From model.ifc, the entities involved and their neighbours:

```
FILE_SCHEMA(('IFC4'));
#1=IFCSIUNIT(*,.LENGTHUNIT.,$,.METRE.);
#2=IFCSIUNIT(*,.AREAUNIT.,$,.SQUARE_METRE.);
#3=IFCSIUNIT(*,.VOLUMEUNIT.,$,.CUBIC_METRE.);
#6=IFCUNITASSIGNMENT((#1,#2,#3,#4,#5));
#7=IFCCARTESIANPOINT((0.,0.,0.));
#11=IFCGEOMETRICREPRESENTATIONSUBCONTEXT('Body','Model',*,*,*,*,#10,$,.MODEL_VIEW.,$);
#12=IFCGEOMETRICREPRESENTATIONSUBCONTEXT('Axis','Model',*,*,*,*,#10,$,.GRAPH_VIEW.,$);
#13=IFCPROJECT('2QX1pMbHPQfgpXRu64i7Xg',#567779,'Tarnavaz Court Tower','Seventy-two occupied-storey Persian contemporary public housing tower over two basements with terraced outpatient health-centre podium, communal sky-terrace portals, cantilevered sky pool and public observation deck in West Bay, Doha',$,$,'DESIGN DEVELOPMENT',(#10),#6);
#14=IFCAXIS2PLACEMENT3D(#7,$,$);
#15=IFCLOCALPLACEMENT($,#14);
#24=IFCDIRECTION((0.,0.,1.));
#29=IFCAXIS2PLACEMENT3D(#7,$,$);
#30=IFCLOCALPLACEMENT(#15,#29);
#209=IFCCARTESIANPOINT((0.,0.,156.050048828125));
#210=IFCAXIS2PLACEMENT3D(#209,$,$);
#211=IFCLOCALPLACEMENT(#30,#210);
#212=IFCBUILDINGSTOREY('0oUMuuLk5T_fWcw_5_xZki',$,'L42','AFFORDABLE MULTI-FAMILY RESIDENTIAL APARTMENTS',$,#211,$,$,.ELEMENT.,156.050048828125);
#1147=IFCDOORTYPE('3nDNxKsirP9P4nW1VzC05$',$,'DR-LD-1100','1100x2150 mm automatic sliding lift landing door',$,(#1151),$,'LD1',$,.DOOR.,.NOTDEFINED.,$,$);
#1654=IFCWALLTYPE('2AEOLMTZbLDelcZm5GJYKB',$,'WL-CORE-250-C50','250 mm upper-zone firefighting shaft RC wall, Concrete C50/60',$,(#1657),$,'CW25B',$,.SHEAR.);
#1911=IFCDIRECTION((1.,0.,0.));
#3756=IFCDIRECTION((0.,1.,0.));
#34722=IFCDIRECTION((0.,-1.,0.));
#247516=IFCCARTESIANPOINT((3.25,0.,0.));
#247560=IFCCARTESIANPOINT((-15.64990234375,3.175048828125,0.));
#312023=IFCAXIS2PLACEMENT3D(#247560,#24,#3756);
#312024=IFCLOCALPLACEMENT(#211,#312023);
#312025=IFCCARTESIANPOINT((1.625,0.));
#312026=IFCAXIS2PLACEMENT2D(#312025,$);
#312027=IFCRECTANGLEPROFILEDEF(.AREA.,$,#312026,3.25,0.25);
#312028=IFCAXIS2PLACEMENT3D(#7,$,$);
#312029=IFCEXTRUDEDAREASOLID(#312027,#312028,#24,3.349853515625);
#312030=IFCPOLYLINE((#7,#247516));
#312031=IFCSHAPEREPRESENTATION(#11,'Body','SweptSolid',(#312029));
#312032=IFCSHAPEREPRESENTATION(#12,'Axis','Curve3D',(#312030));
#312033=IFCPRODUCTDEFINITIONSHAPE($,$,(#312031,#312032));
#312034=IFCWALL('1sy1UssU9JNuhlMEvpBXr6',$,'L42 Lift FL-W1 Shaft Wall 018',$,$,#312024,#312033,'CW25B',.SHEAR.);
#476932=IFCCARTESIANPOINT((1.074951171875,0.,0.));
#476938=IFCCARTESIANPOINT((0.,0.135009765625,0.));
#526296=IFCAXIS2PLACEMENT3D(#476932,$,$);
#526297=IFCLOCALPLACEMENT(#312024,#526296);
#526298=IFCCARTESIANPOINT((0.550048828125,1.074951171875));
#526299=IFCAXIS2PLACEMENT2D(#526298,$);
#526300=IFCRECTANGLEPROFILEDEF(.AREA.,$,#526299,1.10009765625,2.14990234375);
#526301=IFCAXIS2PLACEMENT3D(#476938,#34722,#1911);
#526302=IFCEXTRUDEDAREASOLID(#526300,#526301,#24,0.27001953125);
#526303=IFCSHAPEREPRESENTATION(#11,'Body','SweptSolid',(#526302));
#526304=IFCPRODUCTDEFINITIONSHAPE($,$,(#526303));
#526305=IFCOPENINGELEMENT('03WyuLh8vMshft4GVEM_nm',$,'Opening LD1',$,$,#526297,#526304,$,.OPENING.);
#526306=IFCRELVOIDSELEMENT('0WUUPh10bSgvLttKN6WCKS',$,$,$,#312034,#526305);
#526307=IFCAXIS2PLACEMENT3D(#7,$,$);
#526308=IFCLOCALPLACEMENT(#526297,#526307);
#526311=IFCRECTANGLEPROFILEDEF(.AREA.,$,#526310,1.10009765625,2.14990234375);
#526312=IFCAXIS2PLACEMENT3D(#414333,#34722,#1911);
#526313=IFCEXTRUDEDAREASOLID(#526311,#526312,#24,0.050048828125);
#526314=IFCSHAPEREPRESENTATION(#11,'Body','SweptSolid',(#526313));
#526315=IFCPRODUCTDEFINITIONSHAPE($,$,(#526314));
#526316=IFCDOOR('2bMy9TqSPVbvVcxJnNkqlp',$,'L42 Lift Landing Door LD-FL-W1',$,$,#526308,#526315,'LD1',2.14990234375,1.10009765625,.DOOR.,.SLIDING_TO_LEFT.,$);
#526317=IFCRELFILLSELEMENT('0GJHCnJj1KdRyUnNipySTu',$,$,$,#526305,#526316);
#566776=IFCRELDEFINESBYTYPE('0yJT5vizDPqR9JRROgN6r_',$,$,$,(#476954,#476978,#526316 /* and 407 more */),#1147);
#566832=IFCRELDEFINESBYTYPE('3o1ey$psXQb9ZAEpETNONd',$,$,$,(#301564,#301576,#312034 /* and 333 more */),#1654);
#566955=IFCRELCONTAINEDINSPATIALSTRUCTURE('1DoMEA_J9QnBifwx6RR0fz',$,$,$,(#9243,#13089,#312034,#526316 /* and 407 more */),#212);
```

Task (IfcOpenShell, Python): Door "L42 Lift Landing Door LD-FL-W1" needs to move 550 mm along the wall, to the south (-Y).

```python
import ifcopenshell
import ifcopenshell.api.geometry
import ifcopenshell.util.placement

model = ifcopenshell.open("model.ifc")

door = model.by_id(526316)
opening = door.FillsVoids[0].RelatingOpeningElement
wall = opening.VoidsElements[0].RelatingBuildingElement

wall_matrix = ifcopenshell.util.placement.get_local_placement(wall.ObjectPlacement)
shift = wall_matrix[:3, 0] * -0.55
before = ifcopenshell.util.placement.get_local_placement(door.ObjectPlacement)[:3, 3].copy()

# The door is placed relative to its opening, so it follows when the opening moves.
matrix = ifcopenshell.util.placement.get_local_placement(opening.ObjectPlacement)
matrix[:3, 3] += shift
ifcopenshell.api.geometry.edit_object_placement(
    model, product=opening, matrix=matrix, is_si=False, should_transform_children=True
)

after = ifcopenshell.util.placement.get_local_placement(door.ObjectPlacement)[:3, 3]
print("door moved by", (after - before).round(3) + 0.0)

model.write("model_rev.ifc")
```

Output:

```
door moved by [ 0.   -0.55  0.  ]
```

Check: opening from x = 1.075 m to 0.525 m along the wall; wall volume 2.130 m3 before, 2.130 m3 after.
